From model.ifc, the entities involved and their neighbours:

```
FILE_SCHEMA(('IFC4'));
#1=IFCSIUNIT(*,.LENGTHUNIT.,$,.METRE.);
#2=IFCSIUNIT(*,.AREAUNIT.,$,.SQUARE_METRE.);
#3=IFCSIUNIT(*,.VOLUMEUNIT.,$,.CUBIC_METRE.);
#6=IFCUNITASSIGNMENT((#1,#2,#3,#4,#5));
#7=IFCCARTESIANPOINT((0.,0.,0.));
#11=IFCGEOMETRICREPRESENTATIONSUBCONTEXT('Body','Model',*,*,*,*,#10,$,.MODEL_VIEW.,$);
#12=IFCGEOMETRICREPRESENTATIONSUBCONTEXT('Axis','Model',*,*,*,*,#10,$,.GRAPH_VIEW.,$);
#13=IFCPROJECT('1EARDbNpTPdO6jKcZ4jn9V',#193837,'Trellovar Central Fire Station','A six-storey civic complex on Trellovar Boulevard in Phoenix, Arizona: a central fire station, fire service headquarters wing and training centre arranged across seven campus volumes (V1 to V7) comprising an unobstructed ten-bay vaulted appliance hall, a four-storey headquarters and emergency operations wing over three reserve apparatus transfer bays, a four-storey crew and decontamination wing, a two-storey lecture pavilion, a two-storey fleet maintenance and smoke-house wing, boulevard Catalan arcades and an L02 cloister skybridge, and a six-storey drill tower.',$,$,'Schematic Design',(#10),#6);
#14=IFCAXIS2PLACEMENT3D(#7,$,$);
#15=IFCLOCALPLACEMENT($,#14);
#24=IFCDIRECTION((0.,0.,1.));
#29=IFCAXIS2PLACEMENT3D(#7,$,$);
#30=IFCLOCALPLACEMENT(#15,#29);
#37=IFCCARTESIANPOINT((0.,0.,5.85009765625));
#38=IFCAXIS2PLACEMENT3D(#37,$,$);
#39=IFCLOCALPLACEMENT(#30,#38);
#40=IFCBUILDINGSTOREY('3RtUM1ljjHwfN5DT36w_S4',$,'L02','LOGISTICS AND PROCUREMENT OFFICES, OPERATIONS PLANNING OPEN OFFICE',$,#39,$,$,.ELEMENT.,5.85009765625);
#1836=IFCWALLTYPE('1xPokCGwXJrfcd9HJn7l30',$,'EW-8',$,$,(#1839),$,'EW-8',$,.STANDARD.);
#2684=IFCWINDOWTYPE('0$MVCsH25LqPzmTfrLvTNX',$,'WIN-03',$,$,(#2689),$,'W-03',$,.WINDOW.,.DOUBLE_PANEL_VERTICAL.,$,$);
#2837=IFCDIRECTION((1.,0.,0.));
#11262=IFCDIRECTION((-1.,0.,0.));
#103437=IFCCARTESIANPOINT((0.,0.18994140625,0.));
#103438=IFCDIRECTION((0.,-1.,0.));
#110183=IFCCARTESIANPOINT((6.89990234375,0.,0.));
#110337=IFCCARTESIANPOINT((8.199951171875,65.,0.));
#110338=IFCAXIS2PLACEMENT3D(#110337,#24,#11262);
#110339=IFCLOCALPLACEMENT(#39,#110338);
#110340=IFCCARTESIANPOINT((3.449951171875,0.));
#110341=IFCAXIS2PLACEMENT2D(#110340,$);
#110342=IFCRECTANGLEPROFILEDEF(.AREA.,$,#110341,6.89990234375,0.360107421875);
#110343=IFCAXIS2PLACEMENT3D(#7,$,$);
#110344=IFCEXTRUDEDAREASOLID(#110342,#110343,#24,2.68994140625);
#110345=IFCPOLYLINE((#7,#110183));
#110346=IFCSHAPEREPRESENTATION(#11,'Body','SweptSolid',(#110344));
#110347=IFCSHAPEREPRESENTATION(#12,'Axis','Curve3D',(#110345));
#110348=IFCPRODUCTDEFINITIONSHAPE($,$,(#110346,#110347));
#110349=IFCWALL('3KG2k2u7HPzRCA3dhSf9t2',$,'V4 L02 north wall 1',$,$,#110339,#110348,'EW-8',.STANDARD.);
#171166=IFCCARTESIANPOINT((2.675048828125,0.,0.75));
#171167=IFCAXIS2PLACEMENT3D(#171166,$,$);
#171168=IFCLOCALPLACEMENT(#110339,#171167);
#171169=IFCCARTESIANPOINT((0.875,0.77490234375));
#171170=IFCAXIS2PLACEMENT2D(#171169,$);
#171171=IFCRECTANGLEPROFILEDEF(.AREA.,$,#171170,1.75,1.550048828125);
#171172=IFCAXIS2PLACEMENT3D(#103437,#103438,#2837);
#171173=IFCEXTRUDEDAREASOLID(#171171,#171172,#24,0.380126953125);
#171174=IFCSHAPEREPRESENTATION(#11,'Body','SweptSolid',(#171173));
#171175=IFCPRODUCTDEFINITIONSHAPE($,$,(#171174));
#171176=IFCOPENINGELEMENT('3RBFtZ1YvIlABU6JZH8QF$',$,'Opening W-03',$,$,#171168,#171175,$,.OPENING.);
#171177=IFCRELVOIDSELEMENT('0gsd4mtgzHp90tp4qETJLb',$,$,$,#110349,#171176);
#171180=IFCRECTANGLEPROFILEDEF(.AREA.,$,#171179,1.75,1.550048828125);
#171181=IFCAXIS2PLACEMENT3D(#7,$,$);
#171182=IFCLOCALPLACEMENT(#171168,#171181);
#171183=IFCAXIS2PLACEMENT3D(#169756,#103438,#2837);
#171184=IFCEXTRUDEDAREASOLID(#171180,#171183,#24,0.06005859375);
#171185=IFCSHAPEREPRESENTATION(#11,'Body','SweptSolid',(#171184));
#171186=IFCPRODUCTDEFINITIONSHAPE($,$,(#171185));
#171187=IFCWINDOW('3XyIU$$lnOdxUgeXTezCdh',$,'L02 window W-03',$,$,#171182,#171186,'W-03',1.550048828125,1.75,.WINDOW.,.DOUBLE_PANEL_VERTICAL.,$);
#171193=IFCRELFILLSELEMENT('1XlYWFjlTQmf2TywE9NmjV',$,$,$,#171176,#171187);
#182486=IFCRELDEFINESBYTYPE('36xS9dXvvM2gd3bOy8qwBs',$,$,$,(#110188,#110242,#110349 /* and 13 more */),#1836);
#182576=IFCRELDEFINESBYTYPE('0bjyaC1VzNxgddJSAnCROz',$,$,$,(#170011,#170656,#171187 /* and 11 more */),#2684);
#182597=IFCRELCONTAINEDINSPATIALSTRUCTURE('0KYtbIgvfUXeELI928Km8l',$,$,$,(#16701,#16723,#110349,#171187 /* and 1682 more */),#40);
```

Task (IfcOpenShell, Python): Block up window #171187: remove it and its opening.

```python
import ifcopenshell
import ifcopenshell.api.feature
import ifcopenshell.api.root
import ifcopenshell.geom
import ifcopenshell.util.shape

model = ifcopenshell.open("model.ifc")
settings = ifcopenshell.geom.settings()


def volume(element):
    """Net volume in cubic metres, openings subtracted."""
    shape = ifcopenshell.geom.create_shape(settings, element)
    return ifcopenshell.util.shape.get_volume(shape.geometry)


window = model.by_guid("3XyIU$$lnOdxUgeXTezCdh")
opening = window.FillsVoids[0].RelatingOpeningElement
wall = opening.VoidsElements[0].RelatingBuildingElement
before = volume(wall)

ifcopenshell.api.root.remove_product(model, product=window)
ifcopenshell.api.feature.remove_feature(model, feature=opening)

after = volume(wall)

print(f"wall volume {before:.3f} -> {after:.3f} m3")

model.write("model_edited.ifc")
```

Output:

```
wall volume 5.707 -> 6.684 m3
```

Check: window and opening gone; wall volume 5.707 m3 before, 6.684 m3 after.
